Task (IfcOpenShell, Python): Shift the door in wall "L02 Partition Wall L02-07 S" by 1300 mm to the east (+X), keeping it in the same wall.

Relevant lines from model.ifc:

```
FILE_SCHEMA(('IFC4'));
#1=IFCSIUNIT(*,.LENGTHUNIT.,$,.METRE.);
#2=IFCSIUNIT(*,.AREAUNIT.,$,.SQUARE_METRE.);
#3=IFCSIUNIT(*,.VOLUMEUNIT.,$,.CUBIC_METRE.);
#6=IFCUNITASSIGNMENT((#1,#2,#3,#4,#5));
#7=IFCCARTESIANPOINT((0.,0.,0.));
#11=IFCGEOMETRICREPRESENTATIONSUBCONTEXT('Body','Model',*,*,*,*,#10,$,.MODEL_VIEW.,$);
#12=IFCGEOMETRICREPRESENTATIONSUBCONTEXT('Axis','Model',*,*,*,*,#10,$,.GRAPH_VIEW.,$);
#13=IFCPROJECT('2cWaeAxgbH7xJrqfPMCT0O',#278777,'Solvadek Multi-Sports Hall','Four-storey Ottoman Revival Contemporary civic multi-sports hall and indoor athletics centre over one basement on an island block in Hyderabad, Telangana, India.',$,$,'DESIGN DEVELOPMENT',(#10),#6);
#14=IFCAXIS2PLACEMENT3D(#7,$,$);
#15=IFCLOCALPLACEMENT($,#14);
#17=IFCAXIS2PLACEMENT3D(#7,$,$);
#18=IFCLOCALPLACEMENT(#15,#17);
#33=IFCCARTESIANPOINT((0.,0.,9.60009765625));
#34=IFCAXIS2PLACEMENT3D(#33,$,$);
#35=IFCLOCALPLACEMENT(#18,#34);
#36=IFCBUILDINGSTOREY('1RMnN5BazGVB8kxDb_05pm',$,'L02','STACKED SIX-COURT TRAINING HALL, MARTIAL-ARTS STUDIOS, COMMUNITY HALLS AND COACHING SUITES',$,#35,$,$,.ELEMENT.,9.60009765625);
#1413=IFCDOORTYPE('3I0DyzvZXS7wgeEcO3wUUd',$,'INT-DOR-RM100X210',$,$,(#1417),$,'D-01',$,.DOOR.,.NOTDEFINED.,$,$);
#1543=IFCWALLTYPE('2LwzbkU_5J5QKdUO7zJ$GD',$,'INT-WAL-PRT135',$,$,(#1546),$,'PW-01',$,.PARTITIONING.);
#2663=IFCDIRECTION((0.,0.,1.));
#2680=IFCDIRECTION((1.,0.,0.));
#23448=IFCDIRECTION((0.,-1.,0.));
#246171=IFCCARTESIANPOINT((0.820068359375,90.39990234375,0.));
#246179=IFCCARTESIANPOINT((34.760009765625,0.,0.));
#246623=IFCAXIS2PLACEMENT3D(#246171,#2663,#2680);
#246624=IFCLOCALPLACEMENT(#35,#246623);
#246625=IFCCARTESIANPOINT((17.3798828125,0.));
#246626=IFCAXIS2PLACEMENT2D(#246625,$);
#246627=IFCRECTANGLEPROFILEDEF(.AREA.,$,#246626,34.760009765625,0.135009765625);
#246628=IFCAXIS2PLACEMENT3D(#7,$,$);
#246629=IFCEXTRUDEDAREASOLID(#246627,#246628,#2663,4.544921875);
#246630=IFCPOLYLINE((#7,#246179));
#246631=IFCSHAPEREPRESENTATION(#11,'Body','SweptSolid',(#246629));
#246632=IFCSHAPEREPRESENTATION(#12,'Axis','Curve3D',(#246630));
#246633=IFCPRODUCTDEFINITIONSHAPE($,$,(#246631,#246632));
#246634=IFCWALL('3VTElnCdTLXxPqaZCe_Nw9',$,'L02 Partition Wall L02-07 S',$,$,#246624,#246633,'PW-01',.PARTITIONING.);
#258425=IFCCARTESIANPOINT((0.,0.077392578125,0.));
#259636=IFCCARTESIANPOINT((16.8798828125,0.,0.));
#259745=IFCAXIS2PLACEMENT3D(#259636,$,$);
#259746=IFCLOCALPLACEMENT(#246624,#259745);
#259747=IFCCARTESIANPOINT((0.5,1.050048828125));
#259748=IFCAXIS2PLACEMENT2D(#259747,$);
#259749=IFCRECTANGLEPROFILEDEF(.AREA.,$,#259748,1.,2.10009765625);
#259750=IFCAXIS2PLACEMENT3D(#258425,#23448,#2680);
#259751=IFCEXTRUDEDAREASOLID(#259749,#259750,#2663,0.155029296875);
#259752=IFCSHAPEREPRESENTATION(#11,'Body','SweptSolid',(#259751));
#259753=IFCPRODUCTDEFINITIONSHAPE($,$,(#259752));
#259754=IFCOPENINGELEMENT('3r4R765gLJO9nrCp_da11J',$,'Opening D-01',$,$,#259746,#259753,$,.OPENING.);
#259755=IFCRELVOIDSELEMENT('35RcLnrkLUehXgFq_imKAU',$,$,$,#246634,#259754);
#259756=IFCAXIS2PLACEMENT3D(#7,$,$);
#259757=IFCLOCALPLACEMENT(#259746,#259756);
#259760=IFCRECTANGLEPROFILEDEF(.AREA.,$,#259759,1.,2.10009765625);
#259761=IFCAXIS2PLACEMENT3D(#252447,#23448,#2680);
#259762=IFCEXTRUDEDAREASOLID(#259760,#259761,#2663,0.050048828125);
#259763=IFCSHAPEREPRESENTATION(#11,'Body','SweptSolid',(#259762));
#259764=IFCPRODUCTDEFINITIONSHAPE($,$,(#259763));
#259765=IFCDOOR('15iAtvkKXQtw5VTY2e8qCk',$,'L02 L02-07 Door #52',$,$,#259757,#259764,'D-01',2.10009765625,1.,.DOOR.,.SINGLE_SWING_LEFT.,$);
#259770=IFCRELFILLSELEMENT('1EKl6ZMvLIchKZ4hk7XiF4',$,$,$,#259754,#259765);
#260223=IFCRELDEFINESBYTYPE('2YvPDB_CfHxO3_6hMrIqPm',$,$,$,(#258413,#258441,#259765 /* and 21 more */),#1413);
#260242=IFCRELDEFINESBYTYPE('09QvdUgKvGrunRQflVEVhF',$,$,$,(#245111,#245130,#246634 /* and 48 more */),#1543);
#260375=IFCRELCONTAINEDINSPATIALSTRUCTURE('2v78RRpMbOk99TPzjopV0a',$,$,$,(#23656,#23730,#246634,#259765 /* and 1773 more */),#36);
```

```python
import ifcopenshell
import ifcopenshell.api.geometry
import ifcopenshell.util.placement

model = ifcopenshell.open("model.ifc")

door = model.by_guid("15iAtvkKXQtw5VTY2e8qCk")
opening = door.FillsVoids[0].RelatingOpeningElement
wall = opening.VoidsElements[0].RelatingBuildingElement

wall_matrix = ifcopenshell.util.placement.get_local_placement(wall.ObjectPlacement)
shift = wall_matrix[:3, 0] * 1.3
before = ifcopenshell.util.placement.get_local_placement(door.ObjectPlacement)[:3, 3].copy()

# The door is placed relative to its opening, so it follows when the opening moves.
matrix = ifcopenshell.util.placement.get_local_placement(opening.ObjectPlacement)
matrix[:3, 3] += shift
ifcopenshell.api.geometry.edit_object_placement(
    model, product=opening, matrix=matrix, is_si=False, should_transform_children=True
)

after = ifcopenshell.util.placement.get_local_placement(door.ObjectPlacement)[:3, 3]
print("door moved by", (after - before).round(3) + 0.0)

model.write("model_v2.ifc")
```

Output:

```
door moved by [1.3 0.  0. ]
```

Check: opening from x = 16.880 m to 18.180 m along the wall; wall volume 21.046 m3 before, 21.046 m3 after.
